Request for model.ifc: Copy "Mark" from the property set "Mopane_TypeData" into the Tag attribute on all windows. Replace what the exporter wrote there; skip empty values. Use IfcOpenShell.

First a look at what the model holds.

```python
import ifcopenshell
import ifcopenshell.util.element

model = ifcopenshell.open("model.ifc")
print(model.schema)
windows = model.by_type("IfcWindow")
print(len(windows), "windows")
for e in windows[:8]:
    source = ifcopenshell.util.element.get_pset(e, "Mopane_TypeData", "Mark")
    target = e.Tag
    print(e.id(), repr(source), repr(target), sep=" | ")
```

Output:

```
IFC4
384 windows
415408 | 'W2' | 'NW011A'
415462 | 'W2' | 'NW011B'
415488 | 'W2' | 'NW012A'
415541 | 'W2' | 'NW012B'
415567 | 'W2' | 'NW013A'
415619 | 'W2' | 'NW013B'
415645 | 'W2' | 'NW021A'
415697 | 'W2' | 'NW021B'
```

```python
import ifcopenshell
import ifcopenshell.util.element

model = ifcopenshell.open("model.ifc")

count = 0
for e in model.by_type("IfcWindow"):
    value = ifcopenshell.util.element.get_pset(e, "Mopane_TypeData", "Mark")
    current = e.Tag
    if not value or not value.strip() or current == value:
        continue
    e.Tag = value
    count += 1

print(count, "windows updated")

model.write("model_edited.ifc")
```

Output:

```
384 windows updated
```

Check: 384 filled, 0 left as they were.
